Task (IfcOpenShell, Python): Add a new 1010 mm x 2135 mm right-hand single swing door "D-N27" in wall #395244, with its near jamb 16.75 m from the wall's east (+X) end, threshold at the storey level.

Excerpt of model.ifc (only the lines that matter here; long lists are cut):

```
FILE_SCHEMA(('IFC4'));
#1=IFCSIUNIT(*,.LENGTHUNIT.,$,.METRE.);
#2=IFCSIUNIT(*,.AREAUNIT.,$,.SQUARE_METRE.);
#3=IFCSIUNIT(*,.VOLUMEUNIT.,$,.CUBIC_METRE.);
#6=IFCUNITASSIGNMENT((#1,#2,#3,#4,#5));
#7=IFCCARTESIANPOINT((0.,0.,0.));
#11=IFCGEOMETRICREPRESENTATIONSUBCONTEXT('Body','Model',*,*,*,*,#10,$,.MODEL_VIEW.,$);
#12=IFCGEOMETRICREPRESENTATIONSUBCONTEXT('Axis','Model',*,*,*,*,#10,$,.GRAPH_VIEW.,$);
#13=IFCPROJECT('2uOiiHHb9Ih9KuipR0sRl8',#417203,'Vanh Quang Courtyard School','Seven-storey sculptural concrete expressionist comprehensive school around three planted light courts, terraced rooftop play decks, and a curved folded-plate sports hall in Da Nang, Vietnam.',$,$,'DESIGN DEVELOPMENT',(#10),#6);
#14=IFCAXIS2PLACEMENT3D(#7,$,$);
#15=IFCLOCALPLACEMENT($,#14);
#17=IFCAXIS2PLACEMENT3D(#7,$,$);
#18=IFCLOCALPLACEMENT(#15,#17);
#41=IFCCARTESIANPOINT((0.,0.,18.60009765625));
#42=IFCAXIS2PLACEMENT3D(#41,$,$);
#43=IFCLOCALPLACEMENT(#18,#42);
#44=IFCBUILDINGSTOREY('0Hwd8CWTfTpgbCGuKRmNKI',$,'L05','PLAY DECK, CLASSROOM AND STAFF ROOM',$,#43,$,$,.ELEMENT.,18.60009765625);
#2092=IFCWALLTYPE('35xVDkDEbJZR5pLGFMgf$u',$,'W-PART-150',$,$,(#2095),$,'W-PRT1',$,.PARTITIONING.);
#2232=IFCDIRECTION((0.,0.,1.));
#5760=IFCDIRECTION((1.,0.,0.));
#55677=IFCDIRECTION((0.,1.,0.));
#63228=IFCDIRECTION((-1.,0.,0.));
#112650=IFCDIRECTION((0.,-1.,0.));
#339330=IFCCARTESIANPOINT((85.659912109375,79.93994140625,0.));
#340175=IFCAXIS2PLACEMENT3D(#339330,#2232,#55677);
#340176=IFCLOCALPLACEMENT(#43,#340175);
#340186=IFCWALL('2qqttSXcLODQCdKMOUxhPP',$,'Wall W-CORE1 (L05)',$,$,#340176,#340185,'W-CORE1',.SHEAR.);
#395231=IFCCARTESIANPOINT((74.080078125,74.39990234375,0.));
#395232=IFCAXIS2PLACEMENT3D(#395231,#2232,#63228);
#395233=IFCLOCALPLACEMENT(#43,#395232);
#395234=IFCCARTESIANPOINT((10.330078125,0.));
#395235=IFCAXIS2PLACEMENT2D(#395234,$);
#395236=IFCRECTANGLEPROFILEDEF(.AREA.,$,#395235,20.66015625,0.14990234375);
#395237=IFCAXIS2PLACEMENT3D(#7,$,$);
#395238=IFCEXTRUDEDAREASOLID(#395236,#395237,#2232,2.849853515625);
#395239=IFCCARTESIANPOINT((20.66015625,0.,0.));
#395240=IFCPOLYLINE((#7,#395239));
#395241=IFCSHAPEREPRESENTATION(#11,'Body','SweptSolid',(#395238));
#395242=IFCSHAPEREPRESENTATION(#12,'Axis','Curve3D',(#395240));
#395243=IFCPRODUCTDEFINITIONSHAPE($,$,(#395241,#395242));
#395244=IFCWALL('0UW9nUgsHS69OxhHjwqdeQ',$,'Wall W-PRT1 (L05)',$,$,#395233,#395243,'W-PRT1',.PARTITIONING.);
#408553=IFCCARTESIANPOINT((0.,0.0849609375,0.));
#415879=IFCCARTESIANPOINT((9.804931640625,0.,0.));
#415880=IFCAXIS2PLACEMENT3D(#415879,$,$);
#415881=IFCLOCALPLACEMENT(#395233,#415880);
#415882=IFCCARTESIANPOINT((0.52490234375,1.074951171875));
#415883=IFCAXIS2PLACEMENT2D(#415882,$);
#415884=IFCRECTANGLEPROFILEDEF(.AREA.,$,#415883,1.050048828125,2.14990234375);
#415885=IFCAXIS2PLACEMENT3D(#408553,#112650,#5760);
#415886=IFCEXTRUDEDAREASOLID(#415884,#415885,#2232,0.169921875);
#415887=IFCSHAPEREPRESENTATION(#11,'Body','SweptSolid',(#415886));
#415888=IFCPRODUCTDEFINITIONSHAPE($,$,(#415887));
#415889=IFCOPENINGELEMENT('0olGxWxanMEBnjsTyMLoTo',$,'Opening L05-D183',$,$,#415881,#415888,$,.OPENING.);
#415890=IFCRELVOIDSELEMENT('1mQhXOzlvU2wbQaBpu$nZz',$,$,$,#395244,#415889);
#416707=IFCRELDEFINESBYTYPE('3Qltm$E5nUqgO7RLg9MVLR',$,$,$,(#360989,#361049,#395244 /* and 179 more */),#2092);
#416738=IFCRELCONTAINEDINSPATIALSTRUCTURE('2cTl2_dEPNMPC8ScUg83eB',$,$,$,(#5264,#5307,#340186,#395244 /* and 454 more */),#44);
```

```python
import numpy as np
import ifcopenshell
import ifcopenshell.api.feature
import ifcopenshell.api.geometry
import ifcopenshell.api.root
import ifcopenshell.api.spatial
import ifcopenshell.geom
import ifcopenshell.util.element
import ifcopenshell.util.placement
import ifcopenshell.util.representation
import ifcopenshell.util.shape
import ifcopenshell.util.unit

model = ifcopenshell.open("model.ifc")
unit_scale = ifcopenshell.util.unit.calculate_unit_scale(model)
settings = ifcopenshell.geom.settings()


def volume(element):
    """Net volume in cubic metres, openings subtracted."""
    shape = ifcopenshell.geom.create_shape(settings, element)
    return ifcopenshell.util.shape.get_volume(shape.geometry)


wall = model.by_guid("0UW9nUgsHS69OxhHjwqdeQ")
storey = ifcopenshell.util.element.get_container(wall, ifc_class="IfcBuildingStorey")
context = ifcopenshell.util.representation.get_context(model, "Model", "Body", "MODEL_VIEW")
before = volume(wall)

width, height, from_end, sill = 1.01, 2.135, 16.75, 0.0  # metres

# The wall runs along its own X axis, and the end named is its -X end.
wall_shape = ifcopenshell.geom.create_shape(settings, wall)
x, y, z = ifcopenshell.util.shape.get_vertices(wall_shape.geometry).T
start = x.min() + from_end
face, thickness = float(y.min()), float(y.max() - y.min())
wall_matrix = ifcopenshell.util.placement.get_local_placement(wall.ObjectPlacement)
level = ifcopenshell.util.placement.get_local_placement(storey.ObjectPlacement)[2, 3]


def in_wall(x, y):
    """Placement at x, y metres in the wall's axes, at sill height."""
    matrix = wall_matrix.copy()
    matrix[:, 3] = wall_matrix @ np.array([x / unit_scale, y / unit_scale, 0.0, 1.0])
    matrix[2, 3] = level + sill / unit_scale
    return matrix


# Opening: a box that overshoots both wall faces by 50 mm.
opening = ifcopenshell.api.root.create_entity(model, ifc_class="IfcOpeningElement", predefined_type="OPENING")
box = ifcopenshell.api.geometry.add_wall_representation(
    model, context=context, length=width, height=height, thickness=thickness + 0.1
)
ifcopenshell.api.geometry.assign_representation(model, product=opening, representation=box)
ifcopenshell.api.geometry.edit_object_placement(model, product=opening, matrix=in_wall(start, face - 0.05), is_si=False)
ifcopenshell.api.feature.add_feature(model, feature=opening, element=wall)

door = ifcopenshell.api.root.create_entity(model, ifc_class="IfcDoor", name="D-N27", predefined_type="DOOR")
door.OverallWidth, door.OverallHeight = width / unit_scale, height / unit_scale
door.OperationType = "SINGLE_SWING_RIGHT"
body = ifcopenshell.api.geometry.add_door_representation(
    model,
    context=context,
    overall_width=door.OverallWidth,
    overall_height=door.OverallHeight,
    operation_type="SINGLE_SWING_RIGHT",
    lining_properties={"LiningDepth": thickness / unit_scale, "ThresholdDepth": thickness / unit_scale},
)
ifcopenshell.api.geometry.assign_representation(model, product=door, representation=body)
ifcopenshell.api.spatial.assign_container(model, products=[door], relating_structure=storey)
ifcopenshell.api.feature.add_filling(model, opening=opening, element=door)

# The lining spans the wall, so the door starts at the wall face.
ifcopenshell.api.geometry.edit_object_placement(model, product=door, matrix=in_wall(start, face), is_si=False)

after = volume(wall)

print(f"wall volume {before:.3f} -> {after:.3f} m3")

model.write("model_v2.ifc")
```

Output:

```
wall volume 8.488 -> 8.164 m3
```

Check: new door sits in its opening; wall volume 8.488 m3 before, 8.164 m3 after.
